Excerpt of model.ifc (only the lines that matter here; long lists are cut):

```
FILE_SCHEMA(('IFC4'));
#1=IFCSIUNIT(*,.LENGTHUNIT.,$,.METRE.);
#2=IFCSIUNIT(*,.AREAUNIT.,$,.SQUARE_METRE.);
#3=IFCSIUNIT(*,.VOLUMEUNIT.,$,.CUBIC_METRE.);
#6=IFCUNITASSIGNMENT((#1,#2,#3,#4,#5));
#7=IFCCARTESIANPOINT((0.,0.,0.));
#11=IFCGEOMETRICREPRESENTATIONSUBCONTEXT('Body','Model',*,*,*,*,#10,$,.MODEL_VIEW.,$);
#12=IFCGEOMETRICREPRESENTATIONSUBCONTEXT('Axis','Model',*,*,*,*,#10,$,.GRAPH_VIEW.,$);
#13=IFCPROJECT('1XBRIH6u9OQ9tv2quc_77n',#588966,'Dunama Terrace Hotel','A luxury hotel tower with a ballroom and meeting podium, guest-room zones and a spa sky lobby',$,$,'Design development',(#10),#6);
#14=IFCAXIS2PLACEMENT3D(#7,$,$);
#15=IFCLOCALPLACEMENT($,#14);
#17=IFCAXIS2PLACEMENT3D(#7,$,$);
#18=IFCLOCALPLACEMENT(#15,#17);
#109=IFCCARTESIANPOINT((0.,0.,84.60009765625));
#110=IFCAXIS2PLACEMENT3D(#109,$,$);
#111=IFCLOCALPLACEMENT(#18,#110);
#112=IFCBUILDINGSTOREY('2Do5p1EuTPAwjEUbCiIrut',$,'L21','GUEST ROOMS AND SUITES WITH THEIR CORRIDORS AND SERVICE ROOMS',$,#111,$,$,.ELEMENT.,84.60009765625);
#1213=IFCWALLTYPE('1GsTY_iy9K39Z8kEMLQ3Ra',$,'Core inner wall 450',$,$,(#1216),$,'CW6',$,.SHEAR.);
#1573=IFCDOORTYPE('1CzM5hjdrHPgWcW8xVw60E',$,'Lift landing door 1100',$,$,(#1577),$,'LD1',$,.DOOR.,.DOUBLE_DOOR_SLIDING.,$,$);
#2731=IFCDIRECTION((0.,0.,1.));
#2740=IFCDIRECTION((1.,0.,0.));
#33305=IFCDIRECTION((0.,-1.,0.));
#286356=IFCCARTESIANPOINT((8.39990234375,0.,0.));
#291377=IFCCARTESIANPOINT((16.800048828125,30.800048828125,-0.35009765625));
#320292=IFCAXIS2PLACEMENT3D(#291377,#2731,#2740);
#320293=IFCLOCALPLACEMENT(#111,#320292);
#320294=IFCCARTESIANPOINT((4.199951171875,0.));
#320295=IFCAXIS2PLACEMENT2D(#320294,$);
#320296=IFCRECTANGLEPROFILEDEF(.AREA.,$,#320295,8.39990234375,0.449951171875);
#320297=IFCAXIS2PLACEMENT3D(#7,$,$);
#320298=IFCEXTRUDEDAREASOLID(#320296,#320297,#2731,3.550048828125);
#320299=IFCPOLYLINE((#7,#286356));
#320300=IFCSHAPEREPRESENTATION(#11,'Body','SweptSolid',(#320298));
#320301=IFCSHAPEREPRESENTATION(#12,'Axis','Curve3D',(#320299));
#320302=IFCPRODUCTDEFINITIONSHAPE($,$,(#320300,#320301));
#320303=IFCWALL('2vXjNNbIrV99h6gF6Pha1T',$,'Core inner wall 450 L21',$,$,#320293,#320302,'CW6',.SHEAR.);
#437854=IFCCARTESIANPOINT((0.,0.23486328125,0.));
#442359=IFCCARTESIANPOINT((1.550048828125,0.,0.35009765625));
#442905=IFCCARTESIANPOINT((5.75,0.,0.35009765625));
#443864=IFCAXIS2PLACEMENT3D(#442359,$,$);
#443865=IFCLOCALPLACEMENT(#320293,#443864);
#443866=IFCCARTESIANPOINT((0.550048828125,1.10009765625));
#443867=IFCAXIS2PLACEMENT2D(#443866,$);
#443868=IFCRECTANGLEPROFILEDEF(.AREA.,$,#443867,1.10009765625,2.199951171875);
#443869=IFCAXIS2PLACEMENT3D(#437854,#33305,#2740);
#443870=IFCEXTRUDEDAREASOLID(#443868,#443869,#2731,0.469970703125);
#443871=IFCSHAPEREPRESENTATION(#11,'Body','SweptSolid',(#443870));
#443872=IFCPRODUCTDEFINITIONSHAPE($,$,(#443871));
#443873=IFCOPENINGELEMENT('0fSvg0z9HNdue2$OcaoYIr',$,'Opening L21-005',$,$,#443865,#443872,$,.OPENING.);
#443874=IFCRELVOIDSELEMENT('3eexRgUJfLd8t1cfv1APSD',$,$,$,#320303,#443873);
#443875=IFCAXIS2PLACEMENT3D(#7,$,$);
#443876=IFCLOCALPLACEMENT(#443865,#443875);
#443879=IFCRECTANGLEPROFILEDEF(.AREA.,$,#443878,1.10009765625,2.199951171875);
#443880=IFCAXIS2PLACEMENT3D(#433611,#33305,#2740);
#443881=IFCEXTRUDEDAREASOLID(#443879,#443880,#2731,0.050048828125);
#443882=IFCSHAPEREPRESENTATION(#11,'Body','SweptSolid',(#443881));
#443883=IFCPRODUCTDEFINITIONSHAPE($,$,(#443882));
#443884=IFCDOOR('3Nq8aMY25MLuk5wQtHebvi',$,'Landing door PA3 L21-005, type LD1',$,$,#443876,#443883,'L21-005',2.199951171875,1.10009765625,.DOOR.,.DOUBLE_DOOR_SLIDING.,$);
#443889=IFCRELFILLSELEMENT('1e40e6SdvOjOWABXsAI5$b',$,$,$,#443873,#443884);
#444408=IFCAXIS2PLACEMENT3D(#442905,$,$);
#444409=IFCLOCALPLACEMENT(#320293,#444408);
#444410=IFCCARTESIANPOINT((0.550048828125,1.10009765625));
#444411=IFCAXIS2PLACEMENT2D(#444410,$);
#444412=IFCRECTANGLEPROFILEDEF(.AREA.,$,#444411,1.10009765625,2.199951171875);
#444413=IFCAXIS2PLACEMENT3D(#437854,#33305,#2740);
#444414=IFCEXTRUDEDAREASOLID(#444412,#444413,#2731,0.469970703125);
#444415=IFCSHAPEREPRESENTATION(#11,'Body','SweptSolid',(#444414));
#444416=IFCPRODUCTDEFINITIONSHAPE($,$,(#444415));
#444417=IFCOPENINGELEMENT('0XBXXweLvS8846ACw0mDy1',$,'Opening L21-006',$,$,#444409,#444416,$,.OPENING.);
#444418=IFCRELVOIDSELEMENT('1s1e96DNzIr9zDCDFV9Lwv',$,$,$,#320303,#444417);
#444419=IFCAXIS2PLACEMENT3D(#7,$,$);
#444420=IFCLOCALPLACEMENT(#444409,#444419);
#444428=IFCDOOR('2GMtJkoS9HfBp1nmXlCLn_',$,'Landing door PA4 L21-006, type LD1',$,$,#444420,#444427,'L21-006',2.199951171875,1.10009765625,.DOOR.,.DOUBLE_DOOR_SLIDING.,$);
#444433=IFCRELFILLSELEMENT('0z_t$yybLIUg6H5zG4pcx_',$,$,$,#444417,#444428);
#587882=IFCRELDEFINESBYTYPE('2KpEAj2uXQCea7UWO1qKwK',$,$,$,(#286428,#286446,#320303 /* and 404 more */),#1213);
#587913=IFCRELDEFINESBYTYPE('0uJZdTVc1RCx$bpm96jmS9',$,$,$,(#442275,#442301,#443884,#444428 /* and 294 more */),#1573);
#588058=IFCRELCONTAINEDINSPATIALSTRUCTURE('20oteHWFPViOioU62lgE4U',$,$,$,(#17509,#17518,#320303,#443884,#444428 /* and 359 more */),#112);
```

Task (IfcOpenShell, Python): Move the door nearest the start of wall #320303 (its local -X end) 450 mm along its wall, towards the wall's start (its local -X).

```python
import ifcopenshell
import ifcopenshell.api.geometry
import ifcopenshell.util.placement

model = ifcopenshell.open("model.ifc")

door = model.by_guid("3Nq8aMY25MLuk5wQtHebvi")
opening = door.FillsVoids[0].RelatingOpeningElement
wall = opening.VoidsElements[0].RelatingBuildingElement

wall_matrix = ifcopenshell.util.placement.get_local_placement(wall.ObjectPlacement)
shift = wall_matrix[:3, 0] * -0.45
before = ifcopenshell.util.placement.get_local_placement(door.ObjectPlacement)[:3, 3].copy()

# The door is placed relative to its opening, so it follows when the opening moves.
matrix = ifcopenshell.util.placement.get_local_placement(opening.ObjectPlacement)
matrix[:3, 3] += shift
ifcopenshell.api.geometry.edit_object_placement(
    model, product=opening, matrix=matrix, is_si=False, should_transform_children=True
)

after = ifcopenshell.util.placement.get_local_placement(door.ObjectPlacement)[:3, 3]
print("door moved by", (after - before).round(3) + 0.0)

model.write("model_rev.ifc")
```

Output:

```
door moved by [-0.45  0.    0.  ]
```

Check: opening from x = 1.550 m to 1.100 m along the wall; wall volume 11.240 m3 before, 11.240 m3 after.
